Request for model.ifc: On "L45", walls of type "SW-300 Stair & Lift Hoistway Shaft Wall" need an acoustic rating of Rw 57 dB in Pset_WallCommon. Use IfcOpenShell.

First a look at what the model holds.

```python
import ifcopenshell
import ifcopenshell.util.element

model = ifcopenshell.open("model.ifc")
print(model.schema)
storey = next(s for s in model.by_type("IfcBuildingStorey") if s.Name == "L45")
walls = [e for e in ifcopenshell.util.element.get_decomposition(storey) if e.is_a("IfcWall")]
seen = {}
for e in walls:
    element_type = ifcopenshell.util.element.get_type(e)
    key = (element_type.Name if element_type != e and element_type else None, ifcopenshell.util.element.get_pset(e, "Pset_WallCommon", "AcousticRating"))
    seen[key] = seen.get(key, 0) + 1
for (name, value), count in sorted(seen.items(), key=str):
    print(count, "x", name, "|", value)
```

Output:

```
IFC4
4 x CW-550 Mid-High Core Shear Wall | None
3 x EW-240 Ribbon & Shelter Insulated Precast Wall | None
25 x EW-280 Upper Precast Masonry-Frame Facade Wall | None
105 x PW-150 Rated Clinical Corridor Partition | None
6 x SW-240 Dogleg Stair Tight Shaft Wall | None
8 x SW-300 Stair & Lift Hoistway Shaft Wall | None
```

```python
import ifcopenshell
import ifcopenshell.api.pset
import ifcopenshell.util.element

model = ifcopenshell.open("model.ifc")

storey = next(s for s in model.by_type("IfcBuildingStorey") if s.Name == "L45")
walls = [e for e in ifcopenshell.util.element.get_decomposition(storey) if e.is_a("IfcWall")]

count = 0
for e in walls:
    element_type = ifcopenshell.util.element.get_type(e)
    if element_type in (None, e) or element_type.Name != "SW-300 Stair & Lift Hoistway Shaft Wall":
        continue
    # add_pset returns the element's existing set when there is one.
    pset = ifcopenshell.api.pset.add_pset(model, product=e, name="Pset_WallCommon")
    ifcopenshell.api.pset.edit_pset(model, pset=pset, properties={"AcousticRating": "Rw 57 dB"})
    count += 1

print(count, "walls updated")

model.write("model-out.ifc")
```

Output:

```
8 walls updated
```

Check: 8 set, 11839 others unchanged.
